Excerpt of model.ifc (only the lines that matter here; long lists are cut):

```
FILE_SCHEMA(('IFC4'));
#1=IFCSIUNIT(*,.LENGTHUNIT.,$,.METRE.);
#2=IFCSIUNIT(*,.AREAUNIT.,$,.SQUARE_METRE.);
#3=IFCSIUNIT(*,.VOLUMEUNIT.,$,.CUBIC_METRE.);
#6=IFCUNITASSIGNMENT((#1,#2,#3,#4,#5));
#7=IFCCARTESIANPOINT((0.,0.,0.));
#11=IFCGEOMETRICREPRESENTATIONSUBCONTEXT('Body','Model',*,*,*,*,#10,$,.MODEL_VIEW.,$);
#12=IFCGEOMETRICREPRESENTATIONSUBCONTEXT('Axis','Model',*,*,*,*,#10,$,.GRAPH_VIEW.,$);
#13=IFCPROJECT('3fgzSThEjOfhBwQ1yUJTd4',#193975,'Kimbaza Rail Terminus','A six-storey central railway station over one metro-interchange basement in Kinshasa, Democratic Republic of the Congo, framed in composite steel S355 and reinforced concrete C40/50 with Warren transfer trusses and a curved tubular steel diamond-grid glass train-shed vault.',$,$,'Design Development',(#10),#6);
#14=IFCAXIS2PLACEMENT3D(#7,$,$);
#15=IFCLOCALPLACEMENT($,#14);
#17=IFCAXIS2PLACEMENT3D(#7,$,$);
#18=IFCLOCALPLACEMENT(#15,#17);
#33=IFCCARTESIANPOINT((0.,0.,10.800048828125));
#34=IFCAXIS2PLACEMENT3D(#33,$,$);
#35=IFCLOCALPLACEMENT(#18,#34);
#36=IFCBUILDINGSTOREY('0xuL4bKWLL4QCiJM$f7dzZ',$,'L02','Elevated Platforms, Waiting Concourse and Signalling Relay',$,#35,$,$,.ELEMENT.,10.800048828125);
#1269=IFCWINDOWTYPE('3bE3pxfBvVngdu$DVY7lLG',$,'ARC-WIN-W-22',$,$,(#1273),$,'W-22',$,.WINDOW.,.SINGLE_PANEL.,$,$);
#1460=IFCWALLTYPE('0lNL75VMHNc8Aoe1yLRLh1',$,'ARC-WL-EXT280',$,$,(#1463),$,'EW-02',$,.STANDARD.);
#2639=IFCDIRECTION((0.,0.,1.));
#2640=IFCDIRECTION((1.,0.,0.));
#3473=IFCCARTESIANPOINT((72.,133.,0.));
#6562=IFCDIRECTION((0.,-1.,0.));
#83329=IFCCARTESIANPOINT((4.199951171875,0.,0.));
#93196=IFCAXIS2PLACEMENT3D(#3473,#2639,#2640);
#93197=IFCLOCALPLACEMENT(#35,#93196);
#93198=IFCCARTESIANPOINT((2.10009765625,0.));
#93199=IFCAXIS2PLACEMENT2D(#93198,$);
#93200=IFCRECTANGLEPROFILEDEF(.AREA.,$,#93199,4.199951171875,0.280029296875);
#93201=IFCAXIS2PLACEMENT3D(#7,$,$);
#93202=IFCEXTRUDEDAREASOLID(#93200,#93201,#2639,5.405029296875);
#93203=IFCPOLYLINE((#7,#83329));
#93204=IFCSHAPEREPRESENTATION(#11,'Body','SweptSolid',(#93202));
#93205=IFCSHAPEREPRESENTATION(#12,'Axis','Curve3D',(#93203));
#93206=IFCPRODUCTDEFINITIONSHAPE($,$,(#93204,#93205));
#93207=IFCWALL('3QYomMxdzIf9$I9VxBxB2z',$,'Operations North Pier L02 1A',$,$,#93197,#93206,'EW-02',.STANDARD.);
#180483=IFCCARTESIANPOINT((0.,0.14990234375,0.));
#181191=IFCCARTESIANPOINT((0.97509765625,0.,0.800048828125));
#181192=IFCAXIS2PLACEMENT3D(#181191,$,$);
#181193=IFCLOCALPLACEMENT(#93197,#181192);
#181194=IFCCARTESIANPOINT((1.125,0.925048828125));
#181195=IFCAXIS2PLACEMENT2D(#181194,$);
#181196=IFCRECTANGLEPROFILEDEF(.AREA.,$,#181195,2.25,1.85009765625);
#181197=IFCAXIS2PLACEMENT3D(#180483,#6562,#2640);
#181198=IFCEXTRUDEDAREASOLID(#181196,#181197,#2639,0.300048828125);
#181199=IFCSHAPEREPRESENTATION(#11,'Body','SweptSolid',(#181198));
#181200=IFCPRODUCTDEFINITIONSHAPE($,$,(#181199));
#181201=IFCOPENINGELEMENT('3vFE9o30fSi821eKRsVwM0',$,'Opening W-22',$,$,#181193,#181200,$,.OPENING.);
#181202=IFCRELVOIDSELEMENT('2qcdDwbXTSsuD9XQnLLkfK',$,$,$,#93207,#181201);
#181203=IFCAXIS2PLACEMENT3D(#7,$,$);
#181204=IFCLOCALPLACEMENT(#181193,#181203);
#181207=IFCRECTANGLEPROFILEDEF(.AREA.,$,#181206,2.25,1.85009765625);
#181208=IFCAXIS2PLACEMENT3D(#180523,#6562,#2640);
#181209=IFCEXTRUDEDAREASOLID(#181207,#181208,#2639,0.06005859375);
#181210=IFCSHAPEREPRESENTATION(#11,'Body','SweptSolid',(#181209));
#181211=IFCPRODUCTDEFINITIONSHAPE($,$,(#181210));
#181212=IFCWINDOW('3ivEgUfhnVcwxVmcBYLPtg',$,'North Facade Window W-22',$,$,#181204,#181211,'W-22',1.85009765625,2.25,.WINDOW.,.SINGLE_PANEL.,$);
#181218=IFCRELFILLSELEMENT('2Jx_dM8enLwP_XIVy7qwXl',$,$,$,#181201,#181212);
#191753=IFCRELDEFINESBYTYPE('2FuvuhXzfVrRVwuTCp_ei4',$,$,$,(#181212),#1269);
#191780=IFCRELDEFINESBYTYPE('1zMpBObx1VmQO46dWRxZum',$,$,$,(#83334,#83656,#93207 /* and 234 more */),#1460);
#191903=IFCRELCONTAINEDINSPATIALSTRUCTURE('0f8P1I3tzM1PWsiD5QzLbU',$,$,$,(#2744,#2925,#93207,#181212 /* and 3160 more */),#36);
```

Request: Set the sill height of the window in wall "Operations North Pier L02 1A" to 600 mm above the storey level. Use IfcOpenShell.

```python
import numpy as np
import ifcopenshell
import ifcopenshell.api.geometry
import ifcopenshell.geom
import ifcopenshell.util.element
import ifcopenshell.util.placement
import ifcopenshell.util.shape
import ifcopenshell.util.unit

model = ifcopenshell.open("model.ifc")
unit_scale = ifcopenshell.util.unit.calculate_unit_scale(model)

window = model.by_guid("3ivEgUfhnVcwxVmcBYLPtg")
opening = window.FillsVoids[0].RelatingOpeningElement
storey = ifcopenshell.util.element.get_container(window, ifc_class="IfcBuildingStorey")
level = ifcopenshell.util.placement.get_local_placement(storey.ObjectPlacement)[2, 3]

# The opening's origin need not be at the sill, so measure its lowest point.
shape = ifcopenshell.geom.create_shape(ifcopenshell.geom.settings(), opening)
bottom = ifcopenshell.util.shape.get_shape_bottom_elevation(shape, shape.geometry) / unit_scale
dz = level + 0.6 / unit_scale - bottom

shift = np.array([0.0, 0.0, dz])
# The window is placed relative to its opening, so it follows when the opening moves.
matrix = ifcopenshell.util.placement.get_local_placement(opening.ObjectPlacement)
matrix[:3, 3] += shift
ifcopenshell.api.geometry.edit_object_placement(
    model, product=opening, matrix=matrix, is_si=False, should_transform_children=True
)

print(f"moved by {dz * unit_scale:+.3f} m")

model.write("model-out.ifc")
```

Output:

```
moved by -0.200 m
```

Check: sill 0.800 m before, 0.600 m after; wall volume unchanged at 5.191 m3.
